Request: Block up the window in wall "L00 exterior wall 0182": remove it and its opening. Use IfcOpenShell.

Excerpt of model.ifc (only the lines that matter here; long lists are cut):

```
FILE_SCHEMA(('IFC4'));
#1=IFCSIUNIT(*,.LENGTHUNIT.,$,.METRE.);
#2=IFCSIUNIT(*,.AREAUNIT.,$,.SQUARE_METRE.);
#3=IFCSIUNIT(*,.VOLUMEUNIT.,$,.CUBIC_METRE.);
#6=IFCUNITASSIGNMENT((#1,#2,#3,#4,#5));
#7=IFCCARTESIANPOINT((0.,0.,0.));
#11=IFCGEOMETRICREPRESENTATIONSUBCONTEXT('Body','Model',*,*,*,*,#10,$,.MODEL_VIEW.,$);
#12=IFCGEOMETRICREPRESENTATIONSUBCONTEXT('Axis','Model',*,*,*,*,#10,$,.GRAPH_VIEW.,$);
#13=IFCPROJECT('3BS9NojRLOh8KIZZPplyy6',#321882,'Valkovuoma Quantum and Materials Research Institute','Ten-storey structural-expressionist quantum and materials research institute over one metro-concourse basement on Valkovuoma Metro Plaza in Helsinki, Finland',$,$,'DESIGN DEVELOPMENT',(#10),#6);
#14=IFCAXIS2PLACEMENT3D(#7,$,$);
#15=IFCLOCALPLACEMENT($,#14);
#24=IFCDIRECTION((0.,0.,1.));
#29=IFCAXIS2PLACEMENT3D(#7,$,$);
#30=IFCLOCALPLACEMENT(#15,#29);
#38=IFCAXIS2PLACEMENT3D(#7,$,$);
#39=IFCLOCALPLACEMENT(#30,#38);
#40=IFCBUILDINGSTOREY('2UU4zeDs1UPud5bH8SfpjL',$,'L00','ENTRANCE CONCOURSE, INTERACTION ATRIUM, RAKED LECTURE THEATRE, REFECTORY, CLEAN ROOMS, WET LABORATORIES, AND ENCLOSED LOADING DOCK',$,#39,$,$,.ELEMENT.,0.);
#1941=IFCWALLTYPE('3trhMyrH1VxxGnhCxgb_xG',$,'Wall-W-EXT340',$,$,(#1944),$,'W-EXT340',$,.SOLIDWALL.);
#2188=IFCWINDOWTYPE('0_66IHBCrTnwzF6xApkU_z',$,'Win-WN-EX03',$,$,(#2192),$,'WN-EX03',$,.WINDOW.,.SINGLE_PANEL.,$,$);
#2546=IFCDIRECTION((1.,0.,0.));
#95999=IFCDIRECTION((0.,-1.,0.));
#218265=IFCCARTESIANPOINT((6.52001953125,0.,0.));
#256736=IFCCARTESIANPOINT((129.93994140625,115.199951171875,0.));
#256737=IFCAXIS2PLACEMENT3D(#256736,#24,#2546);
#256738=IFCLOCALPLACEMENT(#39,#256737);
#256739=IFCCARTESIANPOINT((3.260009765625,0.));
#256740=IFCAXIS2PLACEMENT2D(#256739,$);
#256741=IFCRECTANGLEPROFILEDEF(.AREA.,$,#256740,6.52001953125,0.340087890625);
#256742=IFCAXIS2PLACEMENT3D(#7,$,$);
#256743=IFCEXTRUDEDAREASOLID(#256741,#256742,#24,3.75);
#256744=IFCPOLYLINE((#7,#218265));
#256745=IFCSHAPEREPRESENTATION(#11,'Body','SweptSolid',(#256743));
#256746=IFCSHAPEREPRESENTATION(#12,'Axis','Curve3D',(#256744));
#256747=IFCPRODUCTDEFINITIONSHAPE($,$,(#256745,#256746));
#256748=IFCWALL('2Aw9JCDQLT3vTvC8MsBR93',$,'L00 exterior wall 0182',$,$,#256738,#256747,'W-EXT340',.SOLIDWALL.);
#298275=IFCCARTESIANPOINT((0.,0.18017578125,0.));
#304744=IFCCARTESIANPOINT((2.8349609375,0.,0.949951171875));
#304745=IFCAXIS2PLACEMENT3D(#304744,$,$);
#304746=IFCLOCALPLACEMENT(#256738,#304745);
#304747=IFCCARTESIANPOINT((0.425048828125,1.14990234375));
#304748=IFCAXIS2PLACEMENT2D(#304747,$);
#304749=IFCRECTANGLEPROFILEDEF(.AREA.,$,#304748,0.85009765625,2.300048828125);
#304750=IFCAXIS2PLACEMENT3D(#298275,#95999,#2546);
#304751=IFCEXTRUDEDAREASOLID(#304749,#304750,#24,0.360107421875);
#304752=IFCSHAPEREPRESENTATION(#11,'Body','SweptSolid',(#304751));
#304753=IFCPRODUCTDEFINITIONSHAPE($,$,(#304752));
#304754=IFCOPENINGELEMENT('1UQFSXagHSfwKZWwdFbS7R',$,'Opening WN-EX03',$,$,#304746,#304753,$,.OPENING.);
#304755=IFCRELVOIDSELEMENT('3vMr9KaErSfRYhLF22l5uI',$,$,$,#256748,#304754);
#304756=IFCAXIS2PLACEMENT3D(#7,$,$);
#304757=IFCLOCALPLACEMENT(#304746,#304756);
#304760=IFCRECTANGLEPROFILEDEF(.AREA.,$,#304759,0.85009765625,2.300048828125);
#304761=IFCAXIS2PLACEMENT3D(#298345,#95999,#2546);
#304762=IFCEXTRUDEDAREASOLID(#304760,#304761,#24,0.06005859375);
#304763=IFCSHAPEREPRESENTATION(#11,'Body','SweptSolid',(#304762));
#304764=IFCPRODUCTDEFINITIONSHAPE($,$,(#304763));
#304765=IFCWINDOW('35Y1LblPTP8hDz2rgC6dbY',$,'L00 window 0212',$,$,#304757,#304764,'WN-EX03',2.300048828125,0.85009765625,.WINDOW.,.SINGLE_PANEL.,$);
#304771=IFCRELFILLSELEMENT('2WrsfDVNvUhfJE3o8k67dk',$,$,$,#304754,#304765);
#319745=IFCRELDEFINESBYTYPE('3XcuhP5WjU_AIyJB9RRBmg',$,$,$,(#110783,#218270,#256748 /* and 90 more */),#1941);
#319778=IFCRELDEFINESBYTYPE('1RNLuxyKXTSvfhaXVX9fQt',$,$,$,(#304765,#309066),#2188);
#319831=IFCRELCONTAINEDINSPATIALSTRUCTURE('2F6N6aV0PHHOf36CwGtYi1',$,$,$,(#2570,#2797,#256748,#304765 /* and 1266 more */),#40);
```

```python
import ifcopenshell
import ifcopenshell.api.feature
import ifcopenshell.api.root
import ifcopenshell.geom
import ifcopenshell.util.shape

model = ifcopenshell.open("model.ifc")
settings = ifcopenshell.geom.settings()


def volume(element):
    """Net volume in cubic metres, openings subtracted."""
    shape = ifcopenshell.geom.create_shape(settings, element)
    return ifcopenshell.util.shape.get_volume(shape.geometry)


window = model.by_id(304765)
opening = window.FillsVoids[0].RelatingOpeningElement
wall = opening.VoidsElements[0].RelatingBuildingElement
before = volume(wall)

ifcopenshell.api.root.remove_product(model, product=window)
ifcopenshell.api.feature.remove_feature(model, feature=opening)

after = volume(wall)

print(f"wall volume {before:.3f} -> {after:.3f} m3")

model.write("model_rev.ifc")
```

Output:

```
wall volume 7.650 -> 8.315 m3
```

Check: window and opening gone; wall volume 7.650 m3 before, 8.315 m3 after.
